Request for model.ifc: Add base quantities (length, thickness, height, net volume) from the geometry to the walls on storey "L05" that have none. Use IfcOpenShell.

First a look at what the model holds.

```python
import ifcopenshell
import ifcopenshell.util.element
import ifcopenshell.util.unit

model = ifcopenshell.open("model.ifc")
print(model.schema)
for unit_type in ("LENGTHUNIT", "AREAUNIT", "VOLUMEUNIT"):
    print(unit_type, ifcopenshell.util.unit.calculate_unit_scale(model, unit_type))
storey = next(s for s in model.by_type("IfcBuildingStorey") if s.Name == "L05")
walls = [e for e in ifcopenshell.util.element.get_decomposition(storey) if e.is_a("IfcWall")]
for e in sorted(walls, key=lambda e: e.id()):
    print(e.id(), e.is_a(), e.Name, list(ifcopenshell.util.element.get_psets(e, qtos_only=True)), sep=" | ")
```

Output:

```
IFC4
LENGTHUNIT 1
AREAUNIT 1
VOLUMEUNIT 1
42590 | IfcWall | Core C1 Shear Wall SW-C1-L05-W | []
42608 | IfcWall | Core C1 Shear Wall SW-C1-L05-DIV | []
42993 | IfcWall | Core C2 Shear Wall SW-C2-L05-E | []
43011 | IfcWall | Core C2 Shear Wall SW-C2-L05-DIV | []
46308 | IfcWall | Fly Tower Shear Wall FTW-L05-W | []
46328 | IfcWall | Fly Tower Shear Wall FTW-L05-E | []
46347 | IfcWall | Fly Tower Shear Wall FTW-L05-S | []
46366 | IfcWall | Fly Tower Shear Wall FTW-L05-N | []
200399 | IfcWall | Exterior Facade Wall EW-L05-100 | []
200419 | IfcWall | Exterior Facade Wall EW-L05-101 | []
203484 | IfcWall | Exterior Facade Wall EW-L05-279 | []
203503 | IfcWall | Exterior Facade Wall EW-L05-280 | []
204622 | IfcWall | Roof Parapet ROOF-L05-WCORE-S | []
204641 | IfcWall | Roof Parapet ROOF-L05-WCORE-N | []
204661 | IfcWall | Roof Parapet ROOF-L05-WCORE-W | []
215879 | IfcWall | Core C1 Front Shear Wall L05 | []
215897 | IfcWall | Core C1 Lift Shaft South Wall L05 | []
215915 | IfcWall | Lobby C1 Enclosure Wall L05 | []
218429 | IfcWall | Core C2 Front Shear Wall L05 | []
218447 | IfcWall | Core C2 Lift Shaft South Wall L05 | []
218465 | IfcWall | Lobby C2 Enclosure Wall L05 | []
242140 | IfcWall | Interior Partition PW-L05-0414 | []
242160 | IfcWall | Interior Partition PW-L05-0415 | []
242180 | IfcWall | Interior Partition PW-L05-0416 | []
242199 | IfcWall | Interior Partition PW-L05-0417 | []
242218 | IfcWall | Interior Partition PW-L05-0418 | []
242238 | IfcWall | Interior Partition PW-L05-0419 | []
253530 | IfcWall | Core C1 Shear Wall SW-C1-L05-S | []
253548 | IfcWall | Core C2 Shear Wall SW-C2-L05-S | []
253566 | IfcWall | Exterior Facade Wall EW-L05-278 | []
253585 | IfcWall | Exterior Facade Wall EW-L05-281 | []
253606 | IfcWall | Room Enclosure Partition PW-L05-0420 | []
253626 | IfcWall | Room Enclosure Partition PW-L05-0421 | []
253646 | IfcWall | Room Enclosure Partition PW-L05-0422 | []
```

```python
import ifcopenshell
import ifcopenshell.api.pset
import ifcopenshell.geom
import ifcopenshell.util.element
import ifcopenshell.util.shape
import ifcopenshell.util.unit

model = ifcopenshell.open("model.ifc")
unit_scale = ifcopenshell.util.unit.calculate_unit_scale(model)
volume_scale = ifcopenshell.util.unit.calculate_unit_scale(model, "VOLUMEUNIT")
settings = ifcopenshell.geom.settings()

storey = next(s for s in model.by_type("IfcBuildingStorey") if s.Name == "L05")
walls = [e for e in ifcopenshell.util.element.get_decomposition(storey) if e.is_a("IfcWall")]

for e in sorted(walls, key=lambda e: e.id()):
    if ifcopenshell.util.element.get_psets(e, qtos_only=True, should_inherit=False):
        continue
    # Geometry comes back in metres, in the element's own axes.
    shape = ifcopenshell.geom.create_shape(settings, e)
    values = {
        "Length": ifcopenshell.util.shape.get_x(shape.geometry) / unit_scale,
        "Width": ifcopenshell.util.shape.get_y(shape.geometry) / unit_scale,
        "Height": ifcopenshell.util.shape.get_z(shape.geometry) / unit_scale,
        "NetVolume": ifcopenshell.util.shape.get_volume(shape.geometry) / volume_scale,
    }
    qto = ifcopenshell.api.pset.add_qto(model, product=e, name="Qto_WallBaseQuantities")
    ifcopenshell.api.pset.edit_qto(model, qto=qto, properties=values)
    print(e.id(), {k: round(v, 3) for k, v in values.items()})

model.write("model_v2.ifc")
```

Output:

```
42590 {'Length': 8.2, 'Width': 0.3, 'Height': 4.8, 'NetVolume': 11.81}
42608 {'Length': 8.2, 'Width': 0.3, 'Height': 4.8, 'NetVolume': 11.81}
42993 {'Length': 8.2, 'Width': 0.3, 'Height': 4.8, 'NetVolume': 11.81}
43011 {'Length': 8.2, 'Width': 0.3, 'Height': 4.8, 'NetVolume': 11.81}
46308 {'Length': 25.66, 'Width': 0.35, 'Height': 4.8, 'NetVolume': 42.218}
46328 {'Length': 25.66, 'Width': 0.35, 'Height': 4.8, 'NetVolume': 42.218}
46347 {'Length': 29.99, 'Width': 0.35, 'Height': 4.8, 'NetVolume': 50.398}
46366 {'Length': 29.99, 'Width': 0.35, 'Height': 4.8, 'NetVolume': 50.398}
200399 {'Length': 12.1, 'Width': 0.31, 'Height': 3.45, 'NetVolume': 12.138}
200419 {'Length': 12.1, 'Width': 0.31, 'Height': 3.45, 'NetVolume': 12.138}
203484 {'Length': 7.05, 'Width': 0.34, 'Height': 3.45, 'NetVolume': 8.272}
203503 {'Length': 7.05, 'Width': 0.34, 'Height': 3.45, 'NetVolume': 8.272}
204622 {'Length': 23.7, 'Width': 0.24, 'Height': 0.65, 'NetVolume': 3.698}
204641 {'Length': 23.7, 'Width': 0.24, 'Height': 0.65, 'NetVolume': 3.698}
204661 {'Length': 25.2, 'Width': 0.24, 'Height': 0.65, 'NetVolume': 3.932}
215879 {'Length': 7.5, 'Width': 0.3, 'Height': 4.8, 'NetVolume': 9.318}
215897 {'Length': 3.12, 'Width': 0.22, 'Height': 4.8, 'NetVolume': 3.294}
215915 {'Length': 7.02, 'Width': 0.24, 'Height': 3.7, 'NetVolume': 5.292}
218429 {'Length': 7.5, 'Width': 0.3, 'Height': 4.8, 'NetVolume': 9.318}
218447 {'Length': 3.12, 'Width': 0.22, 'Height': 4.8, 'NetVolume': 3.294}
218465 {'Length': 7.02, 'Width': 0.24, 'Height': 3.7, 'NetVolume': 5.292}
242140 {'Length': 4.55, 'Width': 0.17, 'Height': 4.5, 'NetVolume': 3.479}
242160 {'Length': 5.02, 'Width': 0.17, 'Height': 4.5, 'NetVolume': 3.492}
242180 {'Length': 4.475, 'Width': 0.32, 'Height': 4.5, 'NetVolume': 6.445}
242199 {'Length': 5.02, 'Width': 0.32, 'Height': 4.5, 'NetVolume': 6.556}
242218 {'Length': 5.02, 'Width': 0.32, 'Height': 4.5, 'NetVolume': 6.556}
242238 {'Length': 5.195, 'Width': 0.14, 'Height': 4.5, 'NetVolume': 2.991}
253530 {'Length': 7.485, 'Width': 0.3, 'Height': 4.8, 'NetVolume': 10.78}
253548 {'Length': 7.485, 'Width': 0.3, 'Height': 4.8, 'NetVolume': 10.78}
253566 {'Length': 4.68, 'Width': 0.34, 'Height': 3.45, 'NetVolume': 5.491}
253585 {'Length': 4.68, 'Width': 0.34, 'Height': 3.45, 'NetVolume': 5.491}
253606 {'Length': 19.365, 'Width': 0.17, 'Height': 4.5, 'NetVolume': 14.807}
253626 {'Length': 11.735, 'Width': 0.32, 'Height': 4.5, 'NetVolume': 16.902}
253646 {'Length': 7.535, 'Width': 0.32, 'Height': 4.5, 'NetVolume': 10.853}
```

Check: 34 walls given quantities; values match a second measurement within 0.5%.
